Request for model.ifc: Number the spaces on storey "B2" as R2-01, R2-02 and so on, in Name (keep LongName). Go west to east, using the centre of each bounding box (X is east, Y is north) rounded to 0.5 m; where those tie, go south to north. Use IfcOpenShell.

First a look at what the model holds.

```python
import ifcopenshell
import ifcopenshell.util.element
import ifcopenshell.util.placement

model = ifcopenshell.open("model.ifc")
print(model.schema)
storey = next(s for s in model.by_type("IfcBuildingStorey") if s.Name == "B2")
spaces = [e for e in ifcopenshell.util.element.get_decomposition(storey) if e.is_a("IfcSpace")]
for e in sorted(spaces, key=lambda e: e.id()):
    origin = ifcopenshell.util.placement.get_local_placement(e.ObjectPlacement)[:3, 3]
    print(e.id(), e.Name, e.LongName, origin.round(2) + 0.0, sep=" | ")
```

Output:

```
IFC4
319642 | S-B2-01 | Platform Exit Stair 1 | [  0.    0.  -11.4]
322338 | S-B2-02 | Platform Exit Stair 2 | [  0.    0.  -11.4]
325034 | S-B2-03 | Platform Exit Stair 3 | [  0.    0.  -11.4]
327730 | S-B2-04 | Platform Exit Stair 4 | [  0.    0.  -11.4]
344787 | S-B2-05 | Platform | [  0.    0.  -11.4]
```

```python
import ifcopenshell
import ifcopenshell.geom
import ifcopenshell.util.element
import ifcopenshell.util.shape

model = ifcopenshell.open("model.ifc")
settings = ifcopenshell.geom.settings()
settings.set("use-world-coords", True)


def centre(element):
    shape = ifcopenshell.geom.create_shape(settings, element)
    return ifcopenshell.util.shape.get_bbox_centroid(shape.geometry)


storey = next(s for s in model.by_type("IfcBuildingStorey") if s.Name == "B2")
spaces = [e for e in ifcopenshell.util.element.get_decomposition(storey) if e.is_a("IfcSpace")]

# Insertion points can sit at a corner or the storey origin, so sort by the geometry (in metres).
centres = {e: centre(e) for e in spaces}
spaces.sort(key=lambda e: (round(centres[e][0] / 0.5), centres[e][1]))

for i, e in enumerate(spaces, start=1):
    number = f"R2-{i:02d}"
    e.Name = number
    print(e.id(), number)

model.write("model_updated.ifc")
```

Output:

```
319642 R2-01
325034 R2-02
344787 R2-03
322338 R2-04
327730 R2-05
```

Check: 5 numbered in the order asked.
